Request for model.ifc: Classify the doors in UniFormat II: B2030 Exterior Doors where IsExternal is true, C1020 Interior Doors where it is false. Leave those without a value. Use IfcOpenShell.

First a look at what the model holds.

```python
import ifcopenshell
import ifcopenshell.util.element

model = ifcopenshell.open("model.ifc")
print(model.schema)
print("classifications:", [c.Name for c in model.by_type("IfcClassification")])
values = [ifcopenshell.util.element.get_pset(e, "Pset_DoorCommon", "IsExternal") for e in model.by_type("IfcDoor")]
for value in (True, False, None):
    print("IsExternal", value, values.count(value))
```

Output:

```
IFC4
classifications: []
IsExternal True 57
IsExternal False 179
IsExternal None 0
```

```python
import ifcopenshell
import ifcopenshell.api.classification
import ifcopenshell.util.element

model = ifcopenshell.open("model.ifc")

system = ifcopenshell.api.classification.add_classification(model, classification="UniFormat II")

doors = model.by_type("IfcDoor")
external = {e: ifcopenshell.util.element.get_pset(e, "Pset_DoorCommon", "IsExternal") for e in doors}
for flag, code, name in ((True, "B2030", "Exterior Doors"), (False, "C1020", "Interior Doors")):
    products = [e for e in doors if external[e] is flag]
    ifcopenshell.api.classification.add_reference(
        model, products=products, classification=system, identification=code, name=name
    )
    print(code, len(products))

model.write("model_updated.ifc")
```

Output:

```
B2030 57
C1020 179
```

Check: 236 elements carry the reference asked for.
